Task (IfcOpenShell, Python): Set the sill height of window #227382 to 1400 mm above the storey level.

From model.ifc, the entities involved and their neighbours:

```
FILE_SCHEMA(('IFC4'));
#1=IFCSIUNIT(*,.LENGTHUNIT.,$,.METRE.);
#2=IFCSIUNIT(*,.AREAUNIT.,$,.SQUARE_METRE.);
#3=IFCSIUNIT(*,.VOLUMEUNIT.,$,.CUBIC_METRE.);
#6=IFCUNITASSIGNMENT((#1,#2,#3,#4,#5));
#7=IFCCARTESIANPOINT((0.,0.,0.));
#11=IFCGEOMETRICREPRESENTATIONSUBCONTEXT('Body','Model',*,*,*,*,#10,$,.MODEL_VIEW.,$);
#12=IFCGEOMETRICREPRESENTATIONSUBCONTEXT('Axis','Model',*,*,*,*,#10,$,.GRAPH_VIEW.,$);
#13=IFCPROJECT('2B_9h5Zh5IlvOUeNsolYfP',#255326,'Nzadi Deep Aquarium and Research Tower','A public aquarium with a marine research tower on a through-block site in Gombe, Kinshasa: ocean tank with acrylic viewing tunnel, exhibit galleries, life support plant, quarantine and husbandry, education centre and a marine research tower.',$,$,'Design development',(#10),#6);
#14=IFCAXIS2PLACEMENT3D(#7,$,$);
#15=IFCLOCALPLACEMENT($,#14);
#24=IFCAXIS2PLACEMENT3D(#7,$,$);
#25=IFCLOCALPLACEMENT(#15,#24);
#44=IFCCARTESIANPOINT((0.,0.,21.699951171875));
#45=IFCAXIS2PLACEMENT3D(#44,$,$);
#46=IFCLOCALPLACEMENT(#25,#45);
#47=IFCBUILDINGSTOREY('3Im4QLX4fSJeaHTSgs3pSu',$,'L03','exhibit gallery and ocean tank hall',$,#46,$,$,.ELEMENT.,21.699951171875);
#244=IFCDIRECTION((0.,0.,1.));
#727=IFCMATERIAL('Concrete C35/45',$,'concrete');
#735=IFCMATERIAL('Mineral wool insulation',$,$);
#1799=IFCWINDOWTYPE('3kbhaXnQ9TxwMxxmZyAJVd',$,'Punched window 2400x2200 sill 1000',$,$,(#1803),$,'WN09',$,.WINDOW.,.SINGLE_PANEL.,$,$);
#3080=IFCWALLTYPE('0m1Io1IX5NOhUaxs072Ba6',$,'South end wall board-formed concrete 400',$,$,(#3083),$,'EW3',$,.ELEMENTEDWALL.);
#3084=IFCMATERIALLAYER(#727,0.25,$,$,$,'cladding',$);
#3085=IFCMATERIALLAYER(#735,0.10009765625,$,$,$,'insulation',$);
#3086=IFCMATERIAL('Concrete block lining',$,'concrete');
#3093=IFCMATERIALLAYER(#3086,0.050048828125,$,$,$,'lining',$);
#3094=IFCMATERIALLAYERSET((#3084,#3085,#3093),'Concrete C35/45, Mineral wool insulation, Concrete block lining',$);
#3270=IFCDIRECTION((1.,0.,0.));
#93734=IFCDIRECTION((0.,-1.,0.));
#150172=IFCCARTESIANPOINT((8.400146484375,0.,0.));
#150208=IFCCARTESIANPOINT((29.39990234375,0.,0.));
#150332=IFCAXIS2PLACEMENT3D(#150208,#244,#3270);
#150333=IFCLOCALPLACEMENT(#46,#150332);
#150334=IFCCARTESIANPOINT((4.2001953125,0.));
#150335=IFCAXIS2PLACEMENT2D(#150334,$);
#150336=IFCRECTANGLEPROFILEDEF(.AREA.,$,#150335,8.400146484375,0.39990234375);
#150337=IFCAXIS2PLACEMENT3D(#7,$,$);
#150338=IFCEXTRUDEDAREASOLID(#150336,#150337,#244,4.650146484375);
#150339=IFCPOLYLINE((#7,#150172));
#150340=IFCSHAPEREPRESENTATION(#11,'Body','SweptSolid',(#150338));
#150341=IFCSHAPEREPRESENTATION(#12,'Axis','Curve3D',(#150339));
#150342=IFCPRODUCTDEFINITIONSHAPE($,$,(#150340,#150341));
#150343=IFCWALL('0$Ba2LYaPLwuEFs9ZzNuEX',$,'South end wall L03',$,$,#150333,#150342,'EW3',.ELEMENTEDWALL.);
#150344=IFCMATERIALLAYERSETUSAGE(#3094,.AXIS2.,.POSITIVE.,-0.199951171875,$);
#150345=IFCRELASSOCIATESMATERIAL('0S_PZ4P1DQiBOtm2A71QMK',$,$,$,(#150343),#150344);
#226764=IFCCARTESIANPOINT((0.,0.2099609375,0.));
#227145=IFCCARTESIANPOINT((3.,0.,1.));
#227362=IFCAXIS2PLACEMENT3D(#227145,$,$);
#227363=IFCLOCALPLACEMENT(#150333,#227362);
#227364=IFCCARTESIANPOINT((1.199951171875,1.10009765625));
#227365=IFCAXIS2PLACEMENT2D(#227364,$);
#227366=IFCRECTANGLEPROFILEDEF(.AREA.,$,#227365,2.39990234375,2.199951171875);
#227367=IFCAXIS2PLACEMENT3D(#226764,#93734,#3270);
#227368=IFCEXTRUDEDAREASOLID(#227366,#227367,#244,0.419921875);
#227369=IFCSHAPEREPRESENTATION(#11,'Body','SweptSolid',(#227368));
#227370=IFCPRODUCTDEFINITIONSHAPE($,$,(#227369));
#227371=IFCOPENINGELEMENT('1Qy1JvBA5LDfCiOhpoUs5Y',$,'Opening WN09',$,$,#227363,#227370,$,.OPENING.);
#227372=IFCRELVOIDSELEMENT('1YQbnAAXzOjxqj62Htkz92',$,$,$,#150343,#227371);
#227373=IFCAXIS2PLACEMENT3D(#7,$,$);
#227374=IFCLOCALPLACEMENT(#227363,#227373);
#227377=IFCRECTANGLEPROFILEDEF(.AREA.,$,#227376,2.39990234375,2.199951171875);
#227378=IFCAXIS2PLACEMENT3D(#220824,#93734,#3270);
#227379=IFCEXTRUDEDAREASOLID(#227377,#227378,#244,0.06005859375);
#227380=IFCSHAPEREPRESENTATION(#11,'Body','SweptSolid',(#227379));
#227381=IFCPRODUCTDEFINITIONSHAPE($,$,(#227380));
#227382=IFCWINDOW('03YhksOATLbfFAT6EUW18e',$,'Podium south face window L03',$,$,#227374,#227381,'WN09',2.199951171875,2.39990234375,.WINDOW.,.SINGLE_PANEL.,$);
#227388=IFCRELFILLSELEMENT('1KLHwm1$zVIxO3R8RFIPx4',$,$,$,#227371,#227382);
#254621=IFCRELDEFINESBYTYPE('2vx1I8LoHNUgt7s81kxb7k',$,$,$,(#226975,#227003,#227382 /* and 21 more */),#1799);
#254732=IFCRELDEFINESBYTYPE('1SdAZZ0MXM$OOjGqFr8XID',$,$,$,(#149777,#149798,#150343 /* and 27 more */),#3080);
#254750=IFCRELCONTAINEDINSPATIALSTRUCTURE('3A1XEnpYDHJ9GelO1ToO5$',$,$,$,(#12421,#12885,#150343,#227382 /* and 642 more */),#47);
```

```python
import numpy as np
import ifcopenshell
import ifcopenshell.api.geometry
import ifcopenshell.geom
import ifcopenshell.util.element
import ifcopenshell.util.placement
import ifcopenshell.util.shape
import ifcopenshell.util.unit

model = ifcopenshell.open("model.ifc")
unit_scale = ifcopenshell.util.unit.calculate_unit_scale(model)

window = model.by_guid("03YhksOATLbfFAT6EUW18e")
opening = window.FillsVoids[0].RelatingOpeningElement
storey = ifcopenshell.util.element.get_container(window, ifc_class="IfcBuildingStorey")
level = ifcopenshell.util.placement.get_local_placement(storey.ObjectPlacement)[2, 3]

# The opening's origin need not be at the sill, so measure its lowest point.
shape = ifcopenshell.geom.create_shape(ifcopenshell.geom.settings(), opening)
bottom = ifcopenshell.util.shape.get_shape_bottom_elevation(shape, shape.geometry) / unit_scale
dz = level + 1.4 / unit_scale - bottom

shift = np.array([0.0, 0.0, dz])
# The window is placed relative to its opening, so it follows when the opening moves.
matrix = ifcopenshell.util.placement.get_local_placement(opening.ObjectPlacement)
matrix[:3, 3] += shift
ifcopenshell.api.geometry.edit_object_placement(
    model, product=opening, matrix=matrix, is_si=False, should_transform_children=True
)

print(f"moved by {dz * unit_scale:+.3f} m")

model.write("model_v2.ifc")
```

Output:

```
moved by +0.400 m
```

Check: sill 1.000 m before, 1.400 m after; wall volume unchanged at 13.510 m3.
